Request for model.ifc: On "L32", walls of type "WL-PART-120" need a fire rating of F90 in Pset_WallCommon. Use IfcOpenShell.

First a look at what the model holds.

```python
import ifcopenshell
import ifcopenshell.util.element

model = ifcopenshell.open("model.ifc")
print(model.schema)
storey = next(s for s in model.by_type("IfcBuildingStorey") if s.Name == "L32")
walls = [e for e in ifcopenshell.util.element.get_decomposition(storey) if e.is_a("IfcWall")]
seen = {}
for e in walls:
    element_type = ifcopenshell.util.element.get_type(e)
    key = (element_type.Name if element_type != e and element_type else None, ifcopenshell.util.element.get_pset(e, "Pset_WallCommon", "FireRating"))
    seen[key] = seen.get(key, 0) + 1
for (name, value), count in sorted(seen.items(), key=str):
    print(count, "x", name, "|", value)
```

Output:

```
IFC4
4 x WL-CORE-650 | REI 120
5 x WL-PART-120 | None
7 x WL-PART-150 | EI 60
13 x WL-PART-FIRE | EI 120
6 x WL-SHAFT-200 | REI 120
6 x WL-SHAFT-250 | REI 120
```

```python
import ifcopenshell
import ifcopenshell.api.pset
import ifcopenshell.util.element

model = ifcopenshell.open("model.ifc")

storey = next(s for s in model.by_type("IfcBuildingStorey") if s.Name == "L32")
walls = [e for e in ifcopenshell.util.element.get_decomposition(storey) if e.is_a("IfcWall")]

count = 0
for e in walls:
    element_type = ifcopenshell.util.element.get_type(e)
    if element_type in (None, e) or element_type.Name != "WL-PART-120":
        continue
    found = ifcopenshell.util.element.get_pset(e, "Pset_WallCommon", should_inherit=False)
    if found:
        pset = model.by_id(found["id"])
        if len(ifcopenshell.util.element.get_elements_by_pset(pset)) > 1:
            pset = ifcopenshell.api.pset.unshare_pset(model, products=[e], pset=pset)[0]
    else:
        pset = ifcopenshell.api.pset.add_pset(model, product=e, name="Pset_WallCommon")
    ifcopenshell.api.pset.edit_pset(model, pset=pset, properties={"FireRating": "F90"})
    count += 1

print(count, "walls updated")

model.write("model_edited.ifc")
```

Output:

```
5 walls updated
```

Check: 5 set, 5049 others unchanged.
